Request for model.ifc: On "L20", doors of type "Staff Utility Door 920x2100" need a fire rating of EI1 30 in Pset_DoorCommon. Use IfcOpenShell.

First a look at what the model holds.

```python
import ifcopenshell
import ifcopenshell.util.element

model = ifcopenshell.open("model.ifc")
print(model.schema)
storey = next(s for s in model.by_type("IfcBuildingStorey") if s.Name == "L20")
doors = [e for e in ifcopenshell.util.element.get_decomposition(storey) if e.is_a("IfcDoor")]
seen = {}
for e in doors:
    element_type = ifcopenshell.util.element.get_type(e)
    key = (element_type.Name if element_type != e and element_type else None, ifcopenshell.util.element.get_pset(e, "Pset_DoorCommon", "FireRating"))
    seen[key] = seen.get(key, 0) + 1
for (name, value), count in sorted(seen.items(), key=str):
    print(count, "x", name, "|", value)
```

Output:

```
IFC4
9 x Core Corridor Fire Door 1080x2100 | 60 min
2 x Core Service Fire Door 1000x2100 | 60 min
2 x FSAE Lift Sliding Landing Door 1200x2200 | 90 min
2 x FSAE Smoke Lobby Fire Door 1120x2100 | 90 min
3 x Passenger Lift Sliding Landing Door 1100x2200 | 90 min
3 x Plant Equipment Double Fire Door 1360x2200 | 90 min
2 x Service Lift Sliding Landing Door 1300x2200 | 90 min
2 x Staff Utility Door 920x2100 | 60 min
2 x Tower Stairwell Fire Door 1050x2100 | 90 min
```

```python
import ifcopenshell
import ifcopenshell.api.pset
import ifcopenshell.util.element

model = ifcopenshell.open("model.ifc")

storey = next(s for s in model.by_type("IfcBuildingStorey") if s.Name == "L20")
doors = [e for e in ifcopenshell.util.element.get_decomposition(storey) if e.is_a("IfcDoor")]

count = 0
for e in doors:
    element_type = ifcopenshell.util.element.get_type(e)
    if element_type in (None, e) or element_type.Name != "Staff Utility Door 920x2100":
        continue
    # add_pset returns the element's existing set when there is one.
    pset = ifcopenshell.api.pset.add_pset(model, product=e, name="Pset_DoorCommon")
    ifcopenshell.api.pset.edit_pset(model, pset=pset, properties={"FireRating": "EI1 30"})
    count += 1

print(count, "doors updated")

model.write("model_rev.ifc")
```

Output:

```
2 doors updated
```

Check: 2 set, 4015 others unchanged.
